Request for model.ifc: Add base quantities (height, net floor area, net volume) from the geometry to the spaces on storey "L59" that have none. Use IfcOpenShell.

First a look at what the model holds.

```python
import ifcopenshell
import ifcopenshell.util.element
import ifcopenshell.util.unit

model = ifcopenshell.open("model.ifc")
print(model.schema)
for unit_type in ("LENGTHUNIT", "AREAUNIT", "VOLUMEUNIT"):
    print(unit_type, ifcopenshell.util.unit.calculate_unit_scale(model, unit_type))
storey = next(s for s in model.by_type("IfcBuildingStorey") if s.Name == "L59")
spaces = [e for e in ifcopenshell.util.element.get_decomposition(storey) if e.is_a("IfcSpace")]
for e in sorted(spaces, key=lambda e: e.id()):
    print(e.id(), e.is_a(), e.Name, list(ifcopenshell.util.element.get_psets(e, qtos_only=True)), sep=" | ")
```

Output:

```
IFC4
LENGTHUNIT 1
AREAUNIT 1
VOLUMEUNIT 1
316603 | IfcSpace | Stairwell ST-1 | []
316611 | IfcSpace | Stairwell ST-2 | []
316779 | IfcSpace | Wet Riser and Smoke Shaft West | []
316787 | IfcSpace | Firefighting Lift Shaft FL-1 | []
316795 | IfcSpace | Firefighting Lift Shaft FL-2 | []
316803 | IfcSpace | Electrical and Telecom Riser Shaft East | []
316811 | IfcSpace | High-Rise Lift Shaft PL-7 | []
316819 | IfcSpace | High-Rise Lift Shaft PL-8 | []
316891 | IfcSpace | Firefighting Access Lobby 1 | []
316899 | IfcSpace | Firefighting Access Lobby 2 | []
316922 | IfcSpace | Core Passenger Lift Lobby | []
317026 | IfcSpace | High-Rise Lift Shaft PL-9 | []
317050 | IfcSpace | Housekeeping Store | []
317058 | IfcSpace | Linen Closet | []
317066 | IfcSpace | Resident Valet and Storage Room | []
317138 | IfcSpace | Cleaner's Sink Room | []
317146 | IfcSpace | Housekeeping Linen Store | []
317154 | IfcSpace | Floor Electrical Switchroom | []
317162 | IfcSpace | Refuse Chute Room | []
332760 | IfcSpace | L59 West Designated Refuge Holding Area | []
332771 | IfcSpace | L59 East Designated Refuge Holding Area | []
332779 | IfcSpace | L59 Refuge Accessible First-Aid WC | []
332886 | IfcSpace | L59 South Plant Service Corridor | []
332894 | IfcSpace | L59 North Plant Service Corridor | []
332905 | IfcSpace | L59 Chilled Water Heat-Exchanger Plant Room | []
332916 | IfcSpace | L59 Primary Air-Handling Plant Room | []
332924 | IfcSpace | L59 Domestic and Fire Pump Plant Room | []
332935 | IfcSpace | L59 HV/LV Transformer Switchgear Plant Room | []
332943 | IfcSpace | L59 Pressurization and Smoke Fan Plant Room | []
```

```python
import ifcopenshell
import ifcopenshell.api.pset
import ifcopenshell.geom
import ifcopenshell.util.element
import ifcopenshell.util.shape
import ifcopenshell.util.unit

model = ifcopenshell.open("model.ifc")
unit_scale = ifcopenshell.util.unit.calculate_unit_scale(model)
area_scale = ifcopenshell.util.unit.calculate_unit_scale(model, "AREAUNIT")
volume_scale = ifcopenshell.util.unit.calculate_unit_scale(model, "VOLUMEUNIT")
settings = ifcopenshell.geom.settings()

storey = next(s for s in model.by_type("IfcBuildingStorey") if s.Name == "L59")
spaces = [e for e in ifcopenshell.util.element.get_decomposition(storey) if e.is_a("IfcSpace")]

for e in sorted(spaces, key=lambda e: e.id()):
    if ifcopenshell.util.element.get_psets(e, qtos_only=True, should_inherit=False):
        continue
    # Geometry comes back in metres, in the element's own axes.
    shape = ifcopenshell.geom.create_shape(settings, e)
    values = {
        "Height": ifcopenshell.util.shape.get_z(shape.geometry) / unit_scale,
        "NetFloorArea": ifcopenshell.util.shape.get_footprint_area(shape.geometry) / area_scale,
        "NetVolume": ifcopenshell.util.shape.get_volume(shape.geometry) / volume_scale,
    }
    qto = ifcopenshell.api.pset.add_qto(model, product=e, name="Qto_SpaceBaseQuantities")
    ifcopenshell.api.pset.edit_qto(model, qto=qto, properties=values)
    print(e.id(), {k: round(v, 3) for k, v in values.items()})

model.write("model_edited.ifc")
```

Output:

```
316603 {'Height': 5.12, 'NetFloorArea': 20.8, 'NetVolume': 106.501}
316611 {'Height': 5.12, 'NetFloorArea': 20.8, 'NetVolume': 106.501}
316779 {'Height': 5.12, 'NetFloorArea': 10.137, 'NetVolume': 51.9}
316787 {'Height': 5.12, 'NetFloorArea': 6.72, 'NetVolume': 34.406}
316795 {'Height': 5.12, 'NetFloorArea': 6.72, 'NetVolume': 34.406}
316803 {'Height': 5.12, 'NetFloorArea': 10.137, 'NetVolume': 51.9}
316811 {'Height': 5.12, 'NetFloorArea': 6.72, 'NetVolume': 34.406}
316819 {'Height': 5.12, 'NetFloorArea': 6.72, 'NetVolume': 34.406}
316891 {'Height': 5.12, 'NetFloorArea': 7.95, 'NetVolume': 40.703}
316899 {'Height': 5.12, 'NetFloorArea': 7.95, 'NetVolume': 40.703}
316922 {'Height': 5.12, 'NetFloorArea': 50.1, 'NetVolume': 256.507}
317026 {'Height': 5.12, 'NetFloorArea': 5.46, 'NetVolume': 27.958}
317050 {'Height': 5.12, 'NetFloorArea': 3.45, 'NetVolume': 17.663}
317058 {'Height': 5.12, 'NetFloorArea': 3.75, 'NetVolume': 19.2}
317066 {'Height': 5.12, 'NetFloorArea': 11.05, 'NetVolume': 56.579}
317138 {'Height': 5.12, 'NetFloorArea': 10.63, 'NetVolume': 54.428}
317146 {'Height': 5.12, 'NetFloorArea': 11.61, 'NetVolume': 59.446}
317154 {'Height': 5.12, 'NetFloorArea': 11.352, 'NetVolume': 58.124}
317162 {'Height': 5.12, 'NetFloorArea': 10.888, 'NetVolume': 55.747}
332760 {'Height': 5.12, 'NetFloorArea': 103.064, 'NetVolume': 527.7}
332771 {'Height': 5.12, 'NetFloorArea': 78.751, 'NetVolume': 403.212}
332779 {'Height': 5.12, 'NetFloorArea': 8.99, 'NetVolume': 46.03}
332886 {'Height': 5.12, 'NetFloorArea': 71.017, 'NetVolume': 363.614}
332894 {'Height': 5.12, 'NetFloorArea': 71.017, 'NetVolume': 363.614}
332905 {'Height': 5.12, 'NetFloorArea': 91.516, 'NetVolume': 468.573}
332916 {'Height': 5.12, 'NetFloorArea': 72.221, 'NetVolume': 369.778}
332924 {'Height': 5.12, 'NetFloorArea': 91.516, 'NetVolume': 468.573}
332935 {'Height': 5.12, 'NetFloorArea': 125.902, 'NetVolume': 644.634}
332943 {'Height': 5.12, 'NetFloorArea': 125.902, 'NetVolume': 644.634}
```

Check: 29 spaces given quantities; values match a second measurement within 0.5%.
